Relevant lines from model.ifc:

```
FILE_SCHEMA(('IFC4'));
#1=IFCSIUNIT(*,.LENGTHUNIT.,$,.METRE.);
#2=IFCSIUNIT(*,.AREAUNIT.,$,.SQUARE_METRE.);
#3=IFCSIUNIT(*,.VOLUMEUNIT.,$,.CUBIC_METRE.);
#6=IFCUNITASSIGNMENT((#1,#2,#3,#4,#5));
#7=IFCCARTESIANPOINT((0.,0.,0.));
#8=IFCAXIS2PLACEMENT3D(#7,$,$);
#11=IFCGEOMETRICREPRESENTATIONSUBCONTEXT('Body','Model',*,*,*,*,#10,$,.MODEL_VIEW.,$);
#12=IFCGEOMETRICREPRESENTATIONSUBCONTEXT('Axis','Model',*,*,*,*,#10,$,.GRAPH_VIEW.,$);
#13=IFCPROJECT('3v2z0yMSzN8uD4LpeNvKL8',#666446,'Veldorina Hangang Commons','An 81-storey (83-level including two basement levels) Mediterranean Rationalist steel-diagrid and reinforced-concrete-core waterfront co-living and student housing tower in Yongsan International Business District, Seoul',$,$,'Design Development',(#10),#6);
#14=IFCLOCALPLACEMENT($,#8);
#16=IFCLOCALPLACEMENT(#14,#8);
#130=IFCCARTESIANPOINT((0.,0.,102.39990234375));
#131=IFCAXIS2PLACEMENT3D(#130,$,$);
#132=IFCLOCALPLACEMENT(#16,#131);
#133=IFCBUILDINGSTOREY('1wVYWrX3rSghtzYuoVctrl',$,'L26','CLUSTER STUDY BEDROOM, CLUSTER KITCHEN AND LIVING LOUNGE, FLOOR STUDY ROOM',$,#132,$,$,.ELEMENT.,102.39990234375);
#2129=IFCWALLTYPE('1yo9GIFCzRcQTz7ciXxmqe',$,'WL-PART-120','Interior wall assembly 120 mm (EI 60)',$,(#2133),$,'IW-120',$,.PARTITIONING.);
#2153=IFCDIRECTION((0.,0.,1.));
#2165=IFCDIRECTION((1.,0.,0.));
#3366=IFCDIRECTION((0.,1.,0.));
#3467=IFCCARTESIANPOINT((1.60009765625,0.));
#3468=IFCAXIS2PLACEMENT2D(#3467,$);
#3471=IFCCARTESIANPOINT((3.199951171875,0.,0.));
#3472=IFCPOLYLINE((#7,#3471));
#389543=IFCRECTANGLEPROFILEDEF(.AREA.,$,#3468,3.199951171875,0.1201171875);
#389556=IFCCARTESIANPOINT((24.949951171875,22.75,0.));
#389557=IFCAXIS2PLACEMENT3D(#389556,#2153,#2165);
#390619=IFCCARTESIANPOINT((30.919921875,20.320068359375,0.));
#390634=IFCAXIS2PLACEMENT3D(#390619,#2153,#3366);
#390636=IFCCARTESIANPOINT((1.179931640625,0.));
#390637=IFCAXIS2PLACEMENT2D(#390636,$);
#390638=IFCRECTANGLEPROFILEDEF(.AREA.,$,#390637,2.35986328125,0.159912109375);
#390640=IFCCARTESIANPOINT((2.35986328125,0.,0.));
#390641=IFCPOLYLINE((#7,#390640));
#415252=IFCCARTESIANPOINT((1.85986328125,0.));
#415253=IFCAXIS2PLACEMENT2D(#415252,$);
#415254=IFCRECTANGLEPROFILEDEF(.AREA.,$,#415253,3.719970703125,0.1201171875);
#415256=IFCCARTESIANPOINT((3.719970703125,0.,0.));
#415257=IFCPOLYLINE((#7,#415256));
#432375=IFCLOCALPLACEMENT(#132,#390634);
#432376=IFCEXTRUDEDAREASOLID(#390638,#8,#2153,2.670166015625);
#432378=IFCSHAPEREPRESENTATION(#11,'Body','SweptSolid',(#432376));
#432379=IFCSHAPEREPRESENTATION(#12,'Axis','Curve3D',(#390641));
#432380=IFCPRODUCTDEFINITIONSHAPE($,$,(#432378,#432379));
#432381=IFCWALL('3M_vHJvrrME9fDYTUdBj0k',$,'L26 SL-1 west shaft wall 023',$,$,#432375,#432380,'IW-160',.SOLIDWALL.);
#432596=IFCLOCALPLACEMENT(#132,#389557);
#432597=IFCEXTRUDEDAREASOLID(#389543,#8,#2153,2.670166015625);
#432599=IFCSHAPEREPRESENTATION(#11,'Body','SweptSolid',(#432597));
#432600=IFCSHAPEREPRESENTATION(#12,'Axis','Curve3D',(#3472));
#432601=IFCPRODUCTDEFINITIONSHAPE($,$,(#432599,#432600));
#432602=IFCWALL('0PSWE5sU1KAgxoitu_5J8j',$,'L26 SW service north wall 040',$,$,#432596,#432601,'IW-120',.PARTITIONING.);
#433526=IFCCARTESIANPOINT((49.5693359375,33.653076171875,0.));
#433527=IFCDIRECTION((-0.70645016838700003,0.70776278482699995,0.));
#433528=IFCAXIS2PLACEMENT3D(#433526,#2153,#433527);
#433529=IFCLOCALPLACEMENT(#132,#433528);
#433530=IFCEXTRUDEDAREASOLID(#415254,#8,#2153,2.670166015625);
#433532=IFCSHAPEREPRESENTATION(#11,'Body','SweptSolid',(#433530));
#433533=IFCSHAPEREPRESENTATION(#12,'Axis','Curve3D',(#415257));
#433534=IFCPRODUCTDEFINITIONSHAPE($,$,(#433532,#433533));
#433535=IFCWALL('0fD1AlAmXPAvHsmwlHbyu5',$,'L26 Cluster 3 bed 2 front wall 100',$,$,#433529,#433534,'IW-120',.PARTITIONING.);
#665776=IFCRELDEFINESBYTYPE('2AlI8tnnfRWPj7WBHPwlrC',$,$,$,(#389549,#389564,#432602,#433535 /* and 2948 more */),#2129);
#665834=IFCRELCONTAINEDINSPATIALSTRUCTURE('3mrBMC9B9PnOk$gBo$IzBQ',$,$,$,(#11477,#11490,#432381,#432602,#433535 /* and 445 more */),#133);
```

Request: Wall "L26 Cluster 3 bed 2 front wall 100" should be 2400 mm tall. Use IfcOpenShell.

```python
import ifcopenshell
import ifcopenshell.geom
import ifcopenshell.util.representation
import ifcopenshell.util.shape

model = ifcopenshell.open("model.ifc")
settings = ifcopenshell.geom.settings()


def volume(element):
    """Net volume in cubic metres, openings subtracted."""
    shape = ifcopenshell.geom.create_shape(settings, element)
    return ifcopenshell.util.shape.get_volume(shape.geometry)


wall = model.by_id(433535)
before = volume(wall)

body = ifcopenshell.util.representation.get_representation(wall, "Model", "Body")
solid = body.Items[0]
old_height = solid.Depth
solid.Depth = 2.4
after = volume(wall)

print(f"height {old_height:g} -> {solid.Depth:g}, volume {before:.3f} -> {after:.3f} m3")

model.write("model-out.ifc")
```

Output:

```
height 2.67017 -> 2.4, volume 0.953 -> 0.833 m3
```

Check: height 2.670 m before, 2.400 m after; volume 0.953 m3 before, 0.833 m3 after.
